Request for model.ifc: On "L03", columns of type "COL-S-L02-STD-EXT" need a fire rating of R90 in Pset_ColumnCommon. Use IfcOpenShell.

First a look at what the model holds.

```python
import ifcopenshell
import ifcopenshell.util.element

model = ifcopenshell.open("model.ifc")
print(model.schema)
storey = next(s for s in model.by_type("IfcBuildingStorey") if s.Name == "L03")
columns = [e for e in ifcopenshell.util.element.get_decomposition(storey) if e.is_a("IfcColumn")]
seen = {}
for e in columns:
    element_type = ifcopenshell.util.element.get_type(e)
    key = (element_type.Name if element_type != e and element_type else None, ifcopenshell.util.element.get_pset(e, "Pset_ColumnCommon", "FireRating"))
    seen[key] = seen.get(key, 0) + 1
for (name, value), count in sorted(seen.items(), key=str):
    print(count, "x", name, "|", value)
```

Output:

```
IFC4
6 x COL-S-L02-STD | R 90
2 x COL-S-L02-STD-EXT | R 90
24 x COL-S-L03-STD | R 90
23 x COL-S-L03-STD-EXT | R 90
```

```python
import ifcopenshell
import ifcopenshell.api.pset
import ifcopenshell.util.element

model = ifcopenshell.open("model.ifc")

storey = next(s for s in model.by_type("IfcBuildingStorey") if s.Name == "L03")
columns = [e for e in ifcopenshell.util.element.get_decomposition(storey) if e.is_a("IfcColumn")]

count = 0
for e in columns:
    element_type = ifcopenshell.util.element.get_type(e)
    if element_type in (None, e) or element_type.Name != "COL-S-L02-STD-EXT":
        continue
    # add_pset returns the element's existing set when there is one.
    pset = ifcopenshell.api.pset.add_pset(model, product=e, name="Pset_ColumnCommon")
    ifcopenshell.api.pset.edit_pset(model, pset=pset, properties={"FireRating": "R90"})
    count += 1

print(count, "columns updated")

model.write("model_v2.ifc")
```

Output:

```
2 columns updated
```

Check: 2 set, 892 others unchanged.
